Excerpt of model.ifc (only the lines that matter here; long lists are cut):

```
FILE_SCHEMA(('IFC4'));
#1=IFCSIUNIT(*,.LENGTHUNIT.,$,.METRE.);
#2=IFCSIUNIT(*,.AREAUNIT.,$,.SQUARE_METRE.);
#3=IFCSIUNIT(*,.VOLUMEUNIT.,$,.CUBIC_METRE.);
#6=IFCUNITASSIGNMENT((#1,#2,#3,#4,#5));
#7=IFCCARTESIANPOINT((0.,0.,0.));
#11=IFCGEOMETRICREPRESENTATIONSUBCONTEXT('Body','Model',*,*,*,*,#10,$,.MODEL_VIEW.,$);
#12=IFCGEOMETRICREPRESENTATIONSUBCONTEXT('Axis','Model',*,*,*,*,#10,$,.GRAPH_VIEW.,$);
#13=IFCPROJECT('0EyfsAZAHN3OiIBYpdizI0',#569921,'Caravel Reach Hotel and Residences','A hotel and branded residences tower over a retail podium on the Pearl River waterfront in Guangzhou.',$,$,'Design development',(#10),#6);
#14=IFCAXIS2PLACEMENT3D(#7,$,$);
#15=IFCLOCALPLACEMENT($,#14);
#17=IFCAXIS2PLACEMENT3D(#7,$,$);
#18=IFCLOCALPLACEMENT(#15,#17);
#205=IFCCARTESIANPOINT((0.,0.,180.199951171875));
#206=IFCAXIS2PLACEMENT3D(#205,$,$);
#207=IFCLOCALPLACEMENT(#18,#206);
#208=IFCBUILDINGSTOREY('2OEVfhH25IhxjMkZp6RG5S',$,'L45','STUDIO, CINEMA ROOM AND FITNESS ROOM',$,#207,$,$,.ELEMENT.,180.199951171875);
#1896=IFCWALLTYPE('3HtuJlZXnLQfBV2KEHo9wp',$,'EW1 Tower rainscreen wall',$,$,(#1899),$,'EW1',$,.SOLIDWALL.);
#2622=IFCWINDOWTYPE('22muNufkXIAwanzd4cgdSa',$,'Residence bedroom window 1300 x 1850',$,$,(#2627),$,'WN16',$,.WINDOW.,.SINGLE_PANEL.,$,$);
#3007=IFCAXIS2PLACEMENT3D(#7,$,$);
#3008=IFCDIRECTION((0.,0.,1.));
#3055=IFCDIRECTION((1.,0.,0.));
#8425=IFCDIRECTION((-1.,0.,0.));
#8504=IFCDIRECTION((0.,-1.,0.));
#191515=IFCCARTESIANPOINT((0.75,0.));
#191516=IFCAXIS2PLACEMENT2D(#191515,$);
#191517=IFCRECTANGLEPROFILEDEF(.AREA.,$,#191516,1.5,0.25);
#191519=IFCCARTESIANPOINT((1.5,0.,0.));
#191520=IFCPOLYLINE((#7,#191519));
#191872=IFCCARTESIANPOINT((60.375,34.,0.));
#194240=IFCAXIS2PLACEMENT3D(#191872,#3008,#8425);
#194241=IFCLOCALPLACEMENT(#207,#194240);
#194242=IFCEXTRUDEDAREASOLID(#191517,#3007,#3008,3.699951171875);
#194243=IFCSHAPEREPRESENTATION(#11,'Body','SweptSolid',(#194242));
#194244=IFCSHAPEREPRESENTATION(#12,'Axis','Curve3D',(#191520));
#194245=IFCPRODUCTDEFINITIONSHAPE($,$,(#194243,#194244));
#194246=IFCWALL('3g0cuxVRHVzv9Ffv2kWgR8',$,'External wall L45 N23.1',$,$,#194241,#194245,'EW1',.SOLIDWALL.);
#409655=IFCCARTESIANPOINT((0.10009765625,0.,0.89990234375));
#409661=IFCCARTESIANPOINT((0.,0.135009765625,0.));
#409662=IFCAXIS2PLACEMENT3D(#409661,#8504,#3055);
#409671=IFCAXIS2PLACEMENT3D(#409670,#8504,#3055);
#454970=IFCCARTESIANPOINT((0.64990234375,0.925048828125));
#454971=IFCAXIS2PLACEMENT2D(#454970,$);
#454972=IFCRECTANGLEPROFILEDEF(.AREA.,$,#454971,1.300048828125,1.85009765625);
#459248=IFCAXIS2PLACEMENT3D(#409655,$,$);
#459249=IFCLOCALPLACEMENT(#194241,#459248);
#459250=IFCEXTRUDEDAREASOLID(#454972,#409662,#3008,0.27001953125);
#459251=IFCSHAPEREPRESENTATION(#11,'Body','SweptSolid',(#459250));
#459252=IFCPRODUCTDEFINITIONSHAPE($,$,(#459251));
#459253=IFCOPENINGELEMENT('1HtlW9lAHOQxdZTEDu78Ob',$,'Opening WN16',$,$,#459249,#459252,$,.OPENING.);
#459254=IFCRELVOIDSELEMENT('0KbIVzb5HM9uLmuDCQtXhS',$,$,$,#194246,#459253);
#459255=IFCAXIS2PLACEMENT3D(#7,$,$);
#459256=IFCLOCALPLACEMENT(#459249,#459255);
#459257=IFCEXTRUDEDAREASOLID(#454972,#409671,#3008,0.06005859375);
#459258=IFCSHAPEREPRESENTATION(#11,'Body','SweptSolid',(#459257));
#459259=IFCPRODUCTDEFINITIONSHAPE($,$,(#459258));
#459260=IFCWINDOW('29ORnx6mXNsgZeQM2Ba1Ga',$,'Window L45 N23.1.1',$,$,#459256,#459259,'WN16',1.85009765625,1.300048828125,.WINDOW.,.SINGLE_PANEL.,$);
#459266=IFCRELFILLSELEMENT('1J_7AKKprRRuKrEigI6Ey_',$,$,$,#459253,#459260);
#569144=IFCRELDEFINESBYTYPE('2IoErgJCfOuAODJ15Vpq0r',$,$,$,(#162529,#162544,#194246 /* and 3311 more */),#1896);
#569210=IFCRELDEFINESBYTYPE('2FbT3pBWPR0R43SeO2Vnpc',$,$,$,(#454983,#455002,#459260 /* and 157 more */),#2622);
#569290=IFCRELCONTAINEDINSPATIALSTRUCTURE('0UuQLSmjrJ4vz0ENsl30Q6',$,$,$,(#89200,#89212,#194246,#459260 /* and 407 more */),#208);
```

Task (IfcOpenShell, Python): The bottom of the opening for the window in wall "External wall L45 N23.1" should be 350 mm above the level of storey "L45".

```python
import numpy as np
import ifcopenshell
import ifcopenshell.api.geometry
import ifcopenshell.geom
import ifcopenshell.util.element
import ifcopenshell.util.placement
import ifcopenshell.util.shape
import ifcopenshell.util.unit

model = ifcopenshell.open("model.ifc")
unit_scale = ifcopenshell.util.unit.calculate_unit_scale(model)

window = model.by_guid("29ORnx6mXNsgZeQM2Ba1Ga")
opening = window.FillsVoids[0].RelatingOpeningElement
storey = ifcopenshell.util.element.get_container(window, ifc_class="IfcBuildingStorey")
level = ifcopenshell.util.placement.get_local_placement(storey.ObjectPlacement)[2, 3]

# The opening's origin need not be at the sill, so measure its lowest point.
shape = ifcopenshell.geom.create_shape(ifcopenshell.geom.settings(), opening)
bottom = ifcopenshell.util.shape.get_shape_bottom_elevation(shape, shape.geometry) / unit_scale
dz = level + 0.35 / unit_scale - bottom

shift = np.array([0.0, 0.0, dz])
# The window is placed relative to its opening, so it follows when the opening moves.
matrix = ifcopenshell.util.placement.get_local_placement(opening.ObjectPlacement)
matrix[:3, 3] += shift
ifcopenshell.api.geometry.edit_object_placement(
    model, product=opening, matrix=matrix, is_si=False, should_transform_children=True
)

print(f"moved by {dz * unit_scale:+.3f} m")

model.write("model_updated.ifc")
```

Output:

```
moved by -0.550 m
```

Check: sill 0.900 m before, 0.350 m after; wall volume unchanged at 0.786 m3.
